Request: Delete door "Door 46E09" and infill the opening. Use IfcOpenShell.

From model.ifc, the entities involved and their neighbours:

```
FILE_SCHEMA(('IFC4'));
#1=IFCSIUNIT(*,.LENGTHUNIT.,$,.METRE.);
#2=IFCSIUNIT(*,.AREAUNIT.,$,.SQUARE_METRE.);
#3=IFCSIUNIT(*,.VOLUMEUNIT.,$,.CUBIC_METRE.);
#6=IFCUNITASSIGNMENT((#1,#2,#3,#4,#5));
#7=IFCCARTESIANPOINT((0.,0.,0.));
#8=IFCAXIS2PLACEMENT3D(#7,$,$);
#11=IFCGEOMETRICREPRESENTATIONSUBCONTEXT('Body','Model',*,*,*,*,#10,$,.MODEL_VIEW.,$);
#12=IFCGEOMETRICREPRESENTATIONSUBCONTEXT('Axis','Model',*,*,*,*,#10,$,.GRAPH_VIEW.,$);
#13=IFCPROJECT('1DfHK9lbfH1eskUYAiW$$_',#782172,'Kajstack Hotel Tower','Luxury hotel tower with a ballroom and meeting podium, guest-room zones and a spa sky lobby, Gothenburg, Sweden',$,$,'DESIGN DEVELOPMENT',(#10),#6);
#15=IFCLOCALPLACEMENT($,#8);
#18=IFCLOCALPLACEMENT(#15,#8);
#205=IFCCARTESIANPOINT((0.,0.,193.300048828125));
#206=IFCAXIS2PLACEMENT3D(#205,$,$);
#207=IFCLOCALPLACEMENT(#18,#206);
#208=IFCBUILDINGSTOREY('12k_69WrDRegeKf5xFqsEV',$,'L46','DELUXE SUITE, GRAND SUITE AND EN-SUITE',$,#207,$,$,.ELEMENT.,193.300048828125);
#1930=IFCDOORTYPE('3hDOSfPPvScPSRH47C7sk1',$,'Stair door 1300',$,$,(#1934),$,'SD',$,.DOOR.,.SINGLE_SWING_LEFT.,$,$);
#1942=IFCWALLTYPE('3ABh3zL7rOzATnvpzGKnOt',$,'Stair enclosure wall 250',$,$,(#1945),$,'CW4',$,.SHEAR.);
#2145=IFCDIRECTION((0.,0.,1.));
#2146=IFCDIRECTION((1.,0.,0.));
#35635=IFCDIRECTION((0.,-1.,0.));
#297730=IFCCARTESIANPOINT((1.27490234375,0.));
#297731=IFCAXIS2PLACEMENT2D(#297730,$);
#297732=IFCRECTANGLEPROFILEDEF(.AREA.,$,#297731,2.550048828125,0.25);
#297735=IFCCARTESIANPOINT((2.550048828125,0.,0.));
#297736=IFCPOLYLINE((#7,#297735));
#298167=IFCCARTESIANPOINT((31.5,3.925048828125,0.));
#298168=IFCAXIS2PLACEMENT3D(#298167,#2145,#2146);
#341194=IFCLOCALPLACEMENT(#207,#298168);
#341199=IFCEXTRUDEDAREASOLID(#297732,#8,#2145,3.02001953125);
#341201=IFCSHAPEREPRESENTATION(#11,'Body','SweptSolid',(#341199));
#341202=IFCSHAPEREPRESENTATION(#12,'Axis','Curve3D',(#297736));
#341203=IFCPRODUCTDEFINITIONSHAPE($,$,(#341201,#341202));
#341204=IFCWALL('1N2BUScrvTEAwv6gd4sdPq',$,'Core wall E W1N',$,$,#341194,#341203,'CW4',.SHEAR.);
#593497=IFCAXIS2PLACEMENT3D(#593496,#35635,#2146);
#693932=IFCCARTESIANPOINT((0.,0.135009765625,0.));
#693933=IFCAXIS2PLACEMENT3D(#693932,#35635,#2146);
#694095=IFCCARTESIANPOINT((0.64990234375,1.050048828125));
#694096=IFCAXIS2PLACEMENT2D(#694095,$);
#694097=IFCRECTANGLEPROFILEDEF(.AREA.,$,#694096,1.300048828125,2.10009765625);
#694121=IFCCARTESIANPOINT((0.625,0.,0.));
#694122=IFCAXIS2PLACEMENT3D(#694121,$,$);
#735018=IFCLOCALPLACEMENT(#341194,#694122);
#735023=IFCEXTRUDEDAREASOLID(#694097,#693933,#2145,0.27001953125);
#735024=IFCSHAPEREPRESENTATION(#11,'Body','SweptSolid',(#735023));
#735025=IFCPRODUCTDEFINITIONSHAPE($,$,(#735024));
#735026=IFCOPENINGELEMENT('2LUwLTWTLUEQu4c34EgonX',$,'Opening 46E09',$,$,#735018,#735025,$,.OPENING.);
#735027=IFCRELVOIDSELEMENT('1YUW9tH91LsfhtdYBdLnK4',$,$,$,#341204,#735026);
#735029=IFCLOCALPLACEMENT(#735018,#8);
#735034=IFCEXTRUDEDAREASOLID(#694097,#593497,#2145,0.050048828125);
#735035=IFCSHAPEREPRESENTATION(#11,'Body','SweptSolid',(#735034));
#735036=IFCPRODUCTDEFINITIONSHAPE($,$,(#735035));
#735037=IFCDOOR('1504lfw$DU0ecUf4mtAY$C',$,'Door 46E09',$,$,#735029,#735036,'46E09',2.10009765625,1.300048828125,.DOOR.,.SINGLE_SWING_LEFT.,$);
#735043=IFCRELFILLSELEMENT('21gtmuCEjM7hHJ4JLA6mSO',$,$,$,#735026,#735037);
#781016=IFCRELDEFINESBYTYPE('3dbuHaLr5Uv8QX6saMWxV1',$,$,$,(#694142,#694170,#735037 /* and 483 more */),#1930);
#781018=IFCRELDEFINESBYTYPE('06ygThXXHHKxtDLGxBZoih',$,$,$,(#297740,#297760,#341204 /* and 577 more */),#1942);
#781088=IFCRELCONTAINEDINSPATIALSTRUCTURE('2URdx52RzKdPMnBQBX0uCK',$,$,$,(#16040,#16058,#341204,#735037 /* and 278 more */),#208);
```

```python
import ifcopenshell
import ifcopenshell.api.feature
import ifcopenshell.api.root
import ifcopenshell.geom
import ifcopenshell.util.shape

model = ifcopenshell.open("model.ifc")
settings = ifcopenshell.geom.settings()


def volume(element):
    """Net volume in cubic metres, openings subtracted."""
    shape = ifcopenshell.geom.create_shape(settings, element)
    return ifcopenshell.util.shape.get_volume(shape.geometry)


door = model.by_guid("1504lfw$DU0ecUf4mtAY$C")
opening = door.FillsVoids[0].RelatingOpeningElement
wall = opening.VoidsElements[0].RelatingBuildingElement
before = volume(wall)

ifcopenshell.api.root.remove_product(model, product=door)
ifcopenshell.api.feature.remove_feature(model, feature=opening)

after = volume(wall)

print(f"wall volume {before:.3f} -> {after:.3f} m3")

model.write("model_edited.ifc")
```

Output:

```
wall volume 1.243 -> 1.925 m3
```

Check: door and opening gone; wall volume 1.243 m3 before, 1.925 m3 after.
